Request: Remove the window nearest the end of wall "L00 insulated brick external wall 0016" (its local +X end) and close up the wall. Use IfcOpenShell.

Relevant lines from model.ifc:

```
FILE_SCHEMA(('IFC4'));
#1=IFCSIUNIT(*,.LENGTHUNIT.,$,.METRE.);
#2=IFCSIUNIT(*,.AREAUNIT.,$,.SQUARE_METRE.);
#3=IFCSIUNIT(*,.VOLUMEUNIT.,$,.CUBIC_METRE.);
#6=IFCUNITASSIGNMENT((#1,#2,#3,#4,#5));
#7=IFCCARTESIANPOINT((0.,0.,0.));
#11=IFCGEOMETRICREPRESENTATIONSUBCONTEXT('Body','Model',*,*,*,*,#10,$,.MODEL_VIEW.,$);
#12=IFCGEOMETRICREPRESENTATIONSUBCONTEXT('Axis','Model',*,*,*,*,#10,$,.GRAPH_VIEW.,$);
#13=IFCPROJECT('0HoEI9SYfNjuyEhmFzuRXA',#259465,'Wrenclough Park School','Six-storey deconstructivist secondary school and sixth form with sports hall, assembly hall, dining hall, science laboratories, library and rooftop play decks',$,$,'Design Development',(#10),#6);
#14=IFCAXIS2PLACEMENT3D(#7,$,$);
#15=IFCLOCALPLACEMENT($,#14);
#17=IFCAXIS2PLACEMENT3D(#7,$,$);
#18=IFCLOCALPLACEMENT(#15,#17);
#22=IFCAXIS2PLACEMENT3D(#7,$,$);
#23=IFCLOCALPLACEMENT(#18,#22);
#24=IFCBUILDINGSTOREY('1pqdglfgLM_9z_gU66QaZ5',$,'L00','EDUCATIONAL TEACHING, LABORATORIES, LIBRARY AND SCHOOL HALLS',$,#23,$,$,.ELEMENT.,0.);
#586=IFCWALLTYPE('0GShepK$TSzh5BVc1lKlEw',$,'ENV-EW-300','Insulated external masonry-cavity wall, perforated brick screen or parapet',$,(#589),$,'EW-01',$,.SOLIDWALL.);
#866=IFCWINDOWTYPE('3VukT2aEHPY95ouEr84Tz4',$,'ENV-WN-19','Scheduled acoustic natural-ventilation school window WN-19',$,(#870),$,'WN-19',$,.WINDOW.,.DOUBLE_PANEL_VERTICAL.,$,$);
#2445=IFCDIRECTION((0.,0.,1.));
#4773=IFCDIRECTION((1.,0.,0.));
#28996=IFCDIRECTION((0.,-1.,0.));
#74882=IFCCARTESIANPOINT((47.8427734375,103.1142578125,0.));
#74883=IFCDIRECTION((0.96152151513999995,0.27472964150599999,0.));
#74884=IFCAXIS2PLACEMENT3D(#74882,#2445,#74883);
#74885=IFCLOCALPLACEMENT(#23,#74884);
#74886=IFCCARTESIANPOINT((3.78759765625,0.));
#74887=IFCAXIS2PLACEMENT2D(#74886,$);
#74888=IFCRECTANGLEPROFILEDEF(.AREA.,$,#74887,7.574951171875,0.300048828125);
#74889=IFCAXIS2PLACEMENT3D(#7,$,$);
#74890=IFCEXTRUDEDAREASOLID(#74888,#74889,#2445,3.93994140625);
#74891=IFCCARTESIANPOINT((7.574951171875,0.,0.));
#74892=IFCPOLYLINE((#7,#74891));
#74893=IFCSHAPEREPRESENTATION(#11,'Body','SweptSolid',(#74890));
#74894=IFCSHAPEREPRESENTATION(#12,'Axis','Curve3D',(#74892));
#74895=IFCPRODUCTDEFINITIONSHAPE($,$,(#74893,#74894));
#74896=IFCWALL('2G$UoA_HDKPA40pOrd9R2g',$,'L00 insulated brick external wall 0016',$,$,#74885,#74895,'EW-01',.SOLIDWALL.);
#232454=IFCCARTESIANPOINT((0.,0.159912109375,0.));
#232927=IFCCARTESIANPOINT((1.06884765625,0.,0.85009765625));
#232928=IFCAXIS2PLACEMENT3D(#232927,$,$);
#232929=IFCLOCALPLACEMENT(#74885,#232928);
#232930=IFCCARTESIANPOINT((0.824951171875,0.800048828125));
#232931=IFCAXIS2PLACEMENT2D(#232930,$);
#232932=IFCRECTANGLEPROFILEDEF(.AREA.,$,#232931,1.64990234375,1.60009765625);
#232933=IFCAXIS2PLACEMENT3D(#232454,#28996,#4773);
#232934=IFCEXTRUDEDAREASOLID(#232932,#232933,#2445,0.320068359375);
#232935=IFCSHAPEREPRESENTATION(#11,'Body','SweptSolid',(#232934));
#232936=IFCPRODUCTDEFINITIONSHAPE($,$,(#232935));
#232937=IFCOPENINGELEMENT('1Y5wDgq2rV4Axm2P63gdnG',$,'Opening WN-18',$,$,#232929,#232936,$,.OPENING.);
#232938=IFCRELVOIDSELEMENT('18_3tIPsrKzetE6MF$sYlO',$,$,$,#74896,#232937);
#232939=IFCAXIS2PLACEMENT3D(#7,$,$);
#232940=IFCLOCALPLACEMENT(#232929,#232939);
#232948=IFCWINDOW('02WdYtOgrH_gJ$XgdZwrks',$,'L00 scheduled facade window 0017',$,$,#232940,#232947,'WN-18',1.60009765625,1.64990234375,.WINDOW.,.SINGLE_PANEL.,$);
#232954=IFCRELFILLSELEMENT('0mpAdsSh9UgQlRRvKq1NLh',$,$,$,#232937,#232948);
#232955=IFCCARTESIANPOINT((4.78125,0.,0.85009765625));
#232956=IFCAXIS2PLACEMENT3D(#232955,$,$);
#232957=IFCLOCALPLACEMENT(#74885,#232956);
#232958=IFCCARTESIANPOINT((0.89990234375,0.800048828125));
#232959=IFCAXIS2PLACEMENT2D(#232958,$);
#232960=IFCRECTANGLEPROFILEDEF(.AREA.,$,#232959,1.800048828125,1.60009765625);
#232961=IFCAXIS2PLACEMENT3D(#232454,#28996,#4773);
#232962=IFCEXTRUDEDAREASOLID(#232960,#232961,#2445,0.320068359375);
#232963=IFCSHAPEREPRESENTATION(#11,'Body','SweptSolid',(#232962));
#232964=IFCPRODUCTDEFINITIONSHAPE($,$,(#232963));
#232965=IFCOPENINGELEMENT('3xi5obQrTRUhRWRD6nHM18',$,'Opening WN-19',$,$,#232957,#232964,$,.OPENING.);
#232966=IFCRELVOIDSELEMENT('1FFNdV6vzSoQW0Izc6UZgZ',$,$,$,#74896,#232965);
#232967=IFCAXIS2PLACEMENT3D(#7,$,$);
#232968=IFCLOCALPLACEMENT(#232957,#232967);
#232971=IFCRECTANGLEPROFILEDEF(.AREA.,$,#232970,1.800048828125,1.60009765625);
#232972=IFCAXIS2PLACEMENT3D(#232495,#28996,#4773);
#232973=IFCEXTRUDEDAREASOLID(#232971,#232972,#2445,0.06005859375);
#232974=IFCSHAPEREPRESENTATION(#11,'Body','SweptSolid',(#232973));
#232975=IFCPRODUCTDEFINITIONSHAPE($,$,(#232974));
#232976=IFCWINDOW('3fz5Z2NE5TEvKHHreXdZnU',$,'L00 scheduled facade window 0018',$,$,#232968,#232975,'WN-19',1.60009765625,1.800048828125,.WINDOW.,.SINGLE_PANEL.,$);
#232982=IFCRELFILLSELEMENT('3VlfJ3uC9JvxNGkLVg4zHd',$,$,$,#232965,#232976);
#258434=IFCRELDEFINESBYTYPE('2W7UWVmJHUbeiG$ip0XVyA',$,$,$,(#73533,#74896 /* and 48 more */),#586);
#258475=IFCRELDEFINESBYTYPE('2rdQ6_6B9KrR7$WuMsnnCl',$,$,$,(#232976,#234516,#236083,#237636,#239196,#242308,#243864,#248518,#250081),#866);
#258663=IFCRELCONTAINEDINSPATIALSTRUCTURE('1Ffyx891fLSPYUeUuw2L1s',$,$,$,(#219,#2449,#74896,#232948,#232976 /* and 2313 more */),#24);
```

```python
import ifcopenshell
import ifcopenshell.api.feature
import ifcopenshell.api.root
import ifcopenshell.geom
import ifcopenshell.util.shape

model = ifcopenshell.open("model.ifc")
settings = ifcopenshell.geom.settings()


def volume(element):
    """Net volume in cubic metres, openings subtracted."""
    shape = ifcopenshell.geom.create_shape(settings, element)
    return ifcopenshell.util.shape.get_volume(shape.geometry)


window = model.by_id(232976)
opening = window.FillsVoids[0].RelatingOpeningElement
wall = opening.VoidsElements[0].RelatingBuildingElement
before = volume(wall)

ifcopenshell.api.root.remove_product(model, product=window)
ifcopenshell.api.feature.remove_feature(model, feature=opening)

after = volume(wall)

print(f"wall volume {before:.3f} -> {after:.3f} m3")

model.write("model_edited.ifc")
```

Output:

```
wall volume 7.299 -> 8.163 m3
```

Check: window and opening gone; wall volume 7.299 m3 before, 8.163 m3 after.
